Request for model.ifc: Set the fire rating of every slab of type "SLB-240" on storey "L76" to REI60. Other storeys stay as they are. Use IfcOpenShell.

First a look at what the model holds.

```python
import ifcopenshell
import ifcopenshell.util.element

model = ifcopenshell.open("model.ifc")
print(model.schema)
storey = next(s for s in model.by_type("IfcBuildingStorey") if s.Name == "L76")
slabs = [e for e in ifcopenshell.util.element.get_decomposition(storey) if e.is_a("IfcSlab")]
seen = {}
for e in slabs:
    element_type = ifcopenshell.util.element.get_type(e)
    key = (element_type.Name if element_type != e and element_type else None, ifcopenshell.util.element.get_pset(e, "Pset_SlabCommon", "FireRating"))
    seen[key] = seen.get(key, 0) + 1
for (name, value), count in sorted(seen.items(), key=str):
    print(count, "x", name, "|", value)
```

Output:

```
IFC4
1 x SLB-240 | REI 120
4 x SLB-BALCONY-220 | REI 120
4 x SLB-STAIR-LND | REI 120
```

```python
import ifcopenshell
import ifcopenshell.api.pset
import ifcopenshell.util.element

model = ifcopenshell.open("model.ifc")

storey = next(s for s in model.by_type("IfcBuildingStorey") if s.Name == "L76")
slabs = [e for e in ifcopenshell.util.element.get_decomposition(storey) if e.is_a("IfcSlab")]

count = 0
for e in slabs:
    element_type = ifcopenshell.util.element.get_type(e)
    if element_type in (None, e) or element_type.Name != "SLB-240":
        continue
    found = ifcopenshell.util.element.get_pset(e, "Pset_SlabCommon", should_inherit=False)
    if found:
        pset = model.by_id(found["id"])
        if len(ifcopenshell.util.element.get_elements_by_pset(pset)) > 1:
            pset = ifcopenshell.api.pset.unshare_pset(model, products=[e], pset=pset)[0]
    else:
        pset = ifcopenshell.api.pset.add_pset(model, product=e, name="Pset_SlabCommon")
    ifcopenshell.api.pset.edit_pset(model, pset=pset, properties={"FireRating": "REI60"})
    count += 1

print(count, "slabs updated")

model.write("model_edited.ifc")
```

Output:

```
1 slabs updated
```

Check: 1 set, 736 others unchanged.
